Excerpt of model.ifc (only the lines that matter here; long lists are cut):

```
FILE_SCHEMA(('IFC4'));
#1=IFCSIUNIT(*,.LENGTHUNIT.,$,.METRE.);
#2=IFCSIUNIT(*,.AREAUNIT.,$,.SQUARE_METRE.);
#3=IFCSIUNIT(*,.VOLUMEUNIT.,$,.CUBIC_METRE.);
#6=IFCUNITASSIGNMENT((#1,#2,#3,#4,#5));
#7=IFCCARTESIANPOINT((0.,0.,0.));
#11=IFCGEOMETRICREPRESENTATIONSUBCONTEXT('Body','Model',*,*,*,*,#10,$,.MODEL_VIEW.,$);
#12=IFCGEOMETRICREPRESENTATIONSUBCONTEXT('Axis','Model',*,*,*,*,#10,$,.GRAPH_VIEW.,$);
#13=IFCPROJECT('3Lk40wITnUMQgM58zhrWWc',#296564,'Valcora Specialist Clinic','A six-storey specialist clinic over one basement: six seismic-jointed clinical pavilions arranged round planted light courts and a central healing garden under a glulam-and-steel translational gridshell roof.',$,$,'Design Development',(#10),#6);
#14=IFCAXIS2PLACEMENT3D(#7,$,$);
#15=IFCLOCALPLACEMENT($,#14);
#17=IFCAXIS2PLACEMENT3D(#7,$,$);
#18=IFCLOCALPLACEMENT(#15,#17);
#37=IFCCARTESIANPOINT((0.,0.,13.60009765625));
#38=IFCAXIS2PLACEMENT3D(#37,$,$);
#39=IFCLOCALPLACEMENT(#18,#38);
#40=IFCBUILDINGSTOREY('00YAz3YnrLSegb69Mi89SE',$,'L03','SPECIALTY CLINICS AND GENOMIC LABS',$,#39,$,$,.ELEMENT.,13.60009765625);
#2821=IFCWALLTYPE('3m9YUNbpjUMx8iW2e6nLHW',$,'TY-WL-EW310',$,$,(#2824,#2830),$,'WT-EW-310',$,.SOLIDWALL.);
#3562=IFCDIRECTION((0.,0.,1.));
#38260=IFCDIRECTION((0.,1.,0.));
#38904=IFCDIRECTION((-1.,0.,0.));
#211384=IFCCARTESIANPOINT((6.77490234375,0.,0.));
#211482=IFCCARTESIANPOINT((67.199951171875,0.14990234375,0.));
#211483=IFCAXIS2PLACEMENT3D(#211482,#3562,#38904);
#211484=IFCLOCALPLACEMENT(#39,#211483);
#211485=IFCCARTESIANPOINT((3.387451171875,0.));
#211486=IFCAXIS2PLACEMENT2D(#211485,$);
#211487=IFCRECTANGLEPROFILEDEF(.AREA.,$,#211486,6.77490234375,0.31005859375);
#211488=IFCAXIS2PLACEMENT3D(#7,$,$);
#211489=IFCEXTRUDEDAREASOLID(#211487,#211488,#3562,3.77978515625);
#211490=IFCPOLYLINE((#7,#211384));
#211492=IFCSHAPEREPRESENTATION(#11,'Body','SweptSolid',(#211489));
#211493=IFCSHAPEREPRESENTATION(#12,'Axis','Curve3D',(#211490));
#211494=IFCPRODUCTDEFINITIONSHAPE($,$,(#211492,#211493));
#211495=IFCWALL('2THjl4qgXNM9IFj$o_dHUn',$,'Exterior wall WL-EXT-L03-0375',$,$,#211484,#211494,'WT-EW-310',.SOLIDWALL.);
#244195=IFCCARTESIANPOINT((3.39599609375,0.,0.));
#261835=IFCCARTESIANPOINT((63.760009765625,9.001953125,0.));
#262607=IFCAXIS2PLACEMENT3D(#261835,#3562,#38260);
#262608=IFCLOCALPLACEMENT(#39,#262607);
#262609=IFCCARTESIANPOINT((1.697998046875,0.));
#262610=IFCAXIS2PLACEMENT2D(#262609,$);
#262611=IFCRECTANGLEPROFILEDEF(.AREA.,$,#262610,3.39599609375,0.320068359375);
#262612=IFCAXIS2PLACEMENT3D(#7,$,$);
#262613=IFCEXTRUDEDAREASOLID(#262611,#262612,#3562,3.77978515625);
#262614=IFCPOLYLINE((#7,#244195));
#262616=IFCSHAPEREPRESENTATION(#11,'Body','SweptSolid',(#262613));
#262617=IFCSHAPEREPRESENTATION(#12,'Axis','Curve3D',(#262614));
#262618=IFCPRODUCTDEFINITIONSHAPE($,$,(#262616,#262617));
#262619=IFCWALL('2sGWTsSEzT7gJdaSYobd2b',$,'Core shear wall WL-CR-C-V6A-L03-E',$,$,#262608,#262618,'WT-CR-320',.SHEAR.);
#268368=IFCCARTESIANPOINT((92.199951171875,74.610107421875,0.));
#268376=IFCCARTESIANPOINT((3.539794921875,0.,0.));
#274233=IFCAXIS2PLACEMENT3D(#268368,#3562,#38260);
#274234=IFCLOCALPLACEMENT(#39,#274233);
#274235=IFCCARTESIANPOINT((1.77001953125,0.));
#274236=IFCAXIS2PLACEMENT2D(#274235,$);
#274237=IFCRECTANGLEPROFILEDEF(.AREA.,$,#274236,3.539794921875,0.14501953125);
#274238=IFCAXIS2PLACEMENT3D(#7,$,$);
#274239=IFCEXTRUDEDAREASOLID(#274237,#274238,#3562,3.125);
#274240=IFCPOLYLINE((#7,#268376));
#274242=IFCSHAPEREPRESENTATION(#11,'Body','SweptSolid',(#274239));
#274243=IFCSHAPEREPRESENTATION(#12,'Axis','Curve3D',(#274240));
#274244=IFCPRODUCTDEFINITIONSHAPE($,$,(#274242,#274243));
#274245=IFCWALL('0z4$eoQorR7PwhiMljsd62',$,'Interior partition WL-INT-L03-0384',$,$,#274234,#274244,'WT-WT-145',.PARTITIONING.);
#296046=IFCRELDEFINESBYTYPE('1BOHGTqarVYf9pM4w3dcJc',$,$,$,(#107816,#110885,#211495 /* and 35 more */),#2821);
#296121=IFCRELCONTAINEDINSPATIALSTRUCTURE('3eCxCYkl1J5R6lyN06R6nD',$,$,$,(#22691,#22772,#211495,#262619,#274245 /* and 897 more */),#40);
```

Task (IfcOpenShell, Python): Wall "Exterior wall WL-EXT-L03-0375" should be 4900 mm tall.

```python
import ifcopenshell
import ifcopenshell.geom
import ifcopenshell.util.representation
import ifcopenshell.util.shape
import ifcopenshell.util.unit

model = ifcopenshell.open("model.ifc")
unit_scale = ifcopenshell.util.unit.calculate_unit_scale(model)
settings = ifcopenshell.geom.settings()


def volume(element):
    """Net volume in cubic metres, openings subtracted."""
    shape = ifcopenshell.geom.create_shape(settings, element)
    return ifcopenshell.util.shape.get_volume(shape.geometry)


wall = model.by_guid("2THjl4qgXNM9IFj$o_dHUn")
before = volume(wall)

body = ifcopenshell.util.representation.get_representation(wall, "Model", "Body")
solid = body.Items[0]
old_height = solid.Depth
solid.Depth = 4.9 / unit_scale
after = volume(wall)

print(f"height {old_height:g} -> {solid.Depth:g}, volume {before:.3f} -> {after:.3f} m3")

model.write("model_v2.ifc")
```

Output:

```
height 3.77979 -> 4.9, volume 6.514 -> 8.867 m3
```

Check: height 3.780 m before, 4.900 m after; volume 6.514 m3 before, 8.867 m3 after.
